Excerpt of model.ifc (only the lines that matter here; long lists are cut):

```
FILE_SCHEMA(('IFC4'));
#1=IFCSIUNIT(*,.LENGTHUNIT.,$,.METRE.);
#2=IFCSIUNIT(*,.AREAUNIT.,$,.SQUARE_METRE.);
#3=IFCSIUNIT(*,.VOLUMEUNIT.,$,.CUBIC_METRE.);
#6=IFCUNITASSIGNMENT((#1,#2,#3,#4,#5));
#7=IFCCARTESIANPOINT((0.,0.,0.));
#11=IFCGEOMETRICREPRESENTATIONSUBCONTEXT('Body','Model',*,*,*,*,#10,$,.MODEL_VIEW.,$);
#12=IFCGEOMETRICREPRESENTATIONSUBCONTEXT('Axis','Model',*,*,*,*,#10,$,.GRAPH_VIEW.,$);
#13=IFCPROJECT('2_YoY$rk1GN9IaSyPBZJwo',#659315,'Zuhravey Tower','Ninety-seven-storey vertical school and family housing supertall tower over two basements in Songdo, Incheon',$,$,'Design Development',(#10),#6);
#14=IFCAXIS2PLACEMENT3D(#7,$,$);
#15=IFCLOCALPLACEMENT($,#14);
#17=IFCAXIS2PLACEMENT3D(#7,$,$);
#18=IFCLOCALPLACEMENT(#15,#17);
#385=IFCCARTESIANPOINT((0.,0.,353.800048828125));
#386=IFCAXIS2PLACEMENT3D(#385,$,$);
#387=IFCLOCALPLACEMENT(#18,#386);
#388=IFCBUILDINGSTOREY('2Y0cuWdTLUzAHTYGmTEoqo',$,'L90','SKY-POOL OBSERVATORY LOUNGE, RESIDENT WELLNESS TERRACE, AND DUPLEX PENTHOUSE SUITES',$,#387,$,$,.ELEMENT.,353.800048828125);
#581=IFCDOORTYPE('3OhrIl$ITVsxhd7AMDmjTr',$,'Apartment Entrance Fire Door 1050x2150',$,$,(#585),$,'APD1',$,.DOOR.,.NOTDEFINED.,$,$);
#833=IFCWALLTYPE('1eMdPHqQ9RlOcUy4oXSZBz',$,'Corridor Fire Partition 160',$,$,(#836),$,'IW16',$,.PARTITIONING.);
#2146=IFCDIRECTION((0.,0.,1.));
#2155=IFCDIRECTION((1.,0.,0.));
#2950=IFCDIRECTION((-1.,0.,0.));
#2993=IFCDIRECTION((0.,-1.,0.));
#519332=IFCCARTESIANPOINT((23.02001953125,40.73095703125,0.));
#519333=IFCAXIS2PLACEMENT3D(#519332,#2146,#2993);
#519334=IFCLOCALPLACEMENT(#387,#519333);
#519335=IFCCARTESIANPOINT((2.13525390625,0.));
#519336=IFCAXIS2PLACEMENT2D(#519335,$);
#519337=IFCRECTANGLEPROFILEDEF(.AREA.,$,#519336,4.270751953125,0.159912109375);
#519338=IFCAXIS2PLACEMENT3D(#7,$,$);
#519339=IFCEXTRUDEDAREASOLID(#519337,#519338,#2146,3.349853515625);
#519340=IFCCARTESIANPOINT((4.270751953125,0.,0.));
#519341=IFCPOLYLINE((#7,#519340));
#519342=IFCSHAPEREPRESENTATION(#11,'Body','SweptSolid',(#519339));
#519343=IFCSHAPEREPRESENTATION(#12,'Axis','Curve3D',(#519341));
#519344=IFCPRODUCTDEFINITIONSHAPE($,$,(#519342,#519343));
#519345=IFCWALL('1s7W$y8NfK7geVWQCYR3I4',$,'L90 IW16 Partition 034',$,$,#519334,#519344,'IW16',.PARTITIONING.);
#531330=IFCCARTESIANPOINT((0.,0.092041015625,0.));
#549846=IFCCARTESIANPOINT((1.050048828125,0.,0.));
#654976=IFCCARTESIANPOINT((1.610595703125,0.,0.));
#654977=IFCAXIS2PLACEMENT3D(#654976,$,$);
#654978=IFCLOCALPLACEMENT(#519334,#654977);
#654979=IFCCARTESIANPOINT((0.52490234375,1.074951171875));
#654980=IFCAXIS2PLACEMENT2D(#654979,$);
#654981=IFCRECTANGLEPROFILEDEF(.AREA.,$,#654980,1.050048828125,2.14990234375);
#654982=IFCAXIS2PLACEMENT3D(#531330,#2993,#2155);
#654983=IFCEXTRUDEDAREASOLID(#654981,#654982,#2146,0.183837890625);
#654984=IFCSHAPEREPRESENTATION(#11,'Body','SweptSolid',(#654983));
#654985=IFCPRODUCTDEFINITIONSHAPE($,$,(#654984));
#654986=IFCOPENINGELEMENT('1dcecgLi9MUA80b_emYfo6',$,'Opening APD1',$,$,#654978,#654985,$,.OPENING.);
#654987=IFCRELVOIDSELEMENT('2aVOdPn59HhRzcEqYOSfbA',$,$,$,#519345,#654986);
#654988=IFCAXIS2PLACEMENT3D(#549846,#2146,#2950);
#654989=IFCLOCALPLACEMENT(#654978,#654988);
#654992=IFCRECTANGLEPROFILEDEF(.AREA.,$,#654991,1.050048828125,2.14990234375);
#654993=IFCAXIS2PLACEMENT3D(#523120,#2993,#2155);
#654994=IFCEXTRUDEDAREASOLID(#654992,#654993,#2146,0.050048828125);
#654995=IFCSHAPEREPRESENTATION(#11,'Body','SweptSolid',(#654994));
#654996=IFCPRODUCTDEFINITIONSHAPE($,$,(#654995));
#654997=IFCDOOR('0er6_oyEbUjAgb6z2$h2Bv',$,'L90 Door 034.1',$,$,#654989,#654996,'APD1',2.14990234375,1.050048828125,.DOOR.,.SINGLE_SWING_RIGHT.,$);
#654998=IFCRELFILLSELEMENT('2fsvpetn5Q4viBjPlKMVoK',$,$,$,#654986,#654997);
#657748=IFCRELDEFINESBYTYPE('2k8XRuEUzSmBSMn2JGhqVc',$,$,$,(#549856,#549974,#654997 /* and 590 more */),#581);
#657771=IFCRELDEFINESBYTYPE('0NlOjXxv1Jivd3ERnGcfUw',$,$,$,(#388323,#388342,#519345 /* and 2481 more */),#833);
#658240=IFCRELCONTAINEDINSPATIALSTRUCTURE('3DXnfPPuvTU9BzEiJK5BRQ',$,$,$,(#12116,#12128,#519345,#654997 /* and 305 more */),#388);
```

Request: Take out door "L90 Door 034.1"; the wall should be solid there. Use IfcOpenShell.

```python
import ifcopenshell
import ifcopenshell.api.feature
import ifcopenshell.api.root
import ifcopenshell.geom
import ifcopenshell.util.shape

model = ifcopenshell.open("model.ifc")
settings = ifcopenshell.geom.settings()


def volume(element):
    """Net volume in cubic metres, openings subtracted."""
    shape = ifcopenshell.geom.create_shape(settings, element)
    return ifcopenshell.util.shape.get_volume(shape.geometry)


door = model.by_id(654997)
opening = door.FillsVoids[0].RelatingOpeningElement
wall = opening.VoidsElements[0].RelatingBuildingElement
before = volume(wall)

ifcopenshell.api.root.remove_product(model, product=door)
ifcopenshell.api.feature.remove_feature(model, feature=opening)

after = volume(wall)

print(f"wall volume {before:.3f} -> {after:.3f} m3")

model.write("model-out.ifc")
```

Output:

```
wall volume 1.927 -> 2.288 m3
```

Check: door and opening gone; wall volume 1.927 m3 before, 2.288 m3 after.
